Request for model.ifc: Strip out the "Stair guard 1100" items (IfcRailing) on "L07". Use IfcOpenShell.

First a look at what the model holds.

```python
import ifcopenshell
import ifcopenshell.util.element

model = ifcopenshell.open("model.ifc")
print(model.schema)
storey = next(s for s in model.by_type("IfcBuildingStorey") if s.Name == "L07")
railings = [e for e in ifcopenshell.util.element.get_decomposition(storey) if e.is_a("IfcRailing")]
seen = {}
for e in railings:
    element_type = ifcopenshell.util.element.get_type(e)
    name = element_type.Name if element_type not in (None, e) else None
    seen[name] = seen.get(name, 0) + 1
for name, count in sorted(seen.items(), key=str):
    print(count, "x", name)
```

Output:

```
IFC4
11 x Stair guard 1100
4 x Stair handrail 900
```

```python
import ifcopenshell
import ifcopenshell.api.root
import ifcopenshell.util.element

model = ifcopenshell.open("model.ifc")

storey = next(s for s in model.by_type("IfcBuildingStorey") if s.Name == "L07")
railings = [e for e in ifcopenshell.util.element.get_decomposition(storey) if e.is_a("IfcRailing")]
targets = [e for e in railings if (t := ifcopenshell.util.element.get_type(e)) not in (None, e) and t.Name == "Stair guard 1100"]

for e in targets:
    ifcopenshell.api.root.remove_product(model, product=e)
print(len(targets), "removed")

model.write("model_edited.ifc")
```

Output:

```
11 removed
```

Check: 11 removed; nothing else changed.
